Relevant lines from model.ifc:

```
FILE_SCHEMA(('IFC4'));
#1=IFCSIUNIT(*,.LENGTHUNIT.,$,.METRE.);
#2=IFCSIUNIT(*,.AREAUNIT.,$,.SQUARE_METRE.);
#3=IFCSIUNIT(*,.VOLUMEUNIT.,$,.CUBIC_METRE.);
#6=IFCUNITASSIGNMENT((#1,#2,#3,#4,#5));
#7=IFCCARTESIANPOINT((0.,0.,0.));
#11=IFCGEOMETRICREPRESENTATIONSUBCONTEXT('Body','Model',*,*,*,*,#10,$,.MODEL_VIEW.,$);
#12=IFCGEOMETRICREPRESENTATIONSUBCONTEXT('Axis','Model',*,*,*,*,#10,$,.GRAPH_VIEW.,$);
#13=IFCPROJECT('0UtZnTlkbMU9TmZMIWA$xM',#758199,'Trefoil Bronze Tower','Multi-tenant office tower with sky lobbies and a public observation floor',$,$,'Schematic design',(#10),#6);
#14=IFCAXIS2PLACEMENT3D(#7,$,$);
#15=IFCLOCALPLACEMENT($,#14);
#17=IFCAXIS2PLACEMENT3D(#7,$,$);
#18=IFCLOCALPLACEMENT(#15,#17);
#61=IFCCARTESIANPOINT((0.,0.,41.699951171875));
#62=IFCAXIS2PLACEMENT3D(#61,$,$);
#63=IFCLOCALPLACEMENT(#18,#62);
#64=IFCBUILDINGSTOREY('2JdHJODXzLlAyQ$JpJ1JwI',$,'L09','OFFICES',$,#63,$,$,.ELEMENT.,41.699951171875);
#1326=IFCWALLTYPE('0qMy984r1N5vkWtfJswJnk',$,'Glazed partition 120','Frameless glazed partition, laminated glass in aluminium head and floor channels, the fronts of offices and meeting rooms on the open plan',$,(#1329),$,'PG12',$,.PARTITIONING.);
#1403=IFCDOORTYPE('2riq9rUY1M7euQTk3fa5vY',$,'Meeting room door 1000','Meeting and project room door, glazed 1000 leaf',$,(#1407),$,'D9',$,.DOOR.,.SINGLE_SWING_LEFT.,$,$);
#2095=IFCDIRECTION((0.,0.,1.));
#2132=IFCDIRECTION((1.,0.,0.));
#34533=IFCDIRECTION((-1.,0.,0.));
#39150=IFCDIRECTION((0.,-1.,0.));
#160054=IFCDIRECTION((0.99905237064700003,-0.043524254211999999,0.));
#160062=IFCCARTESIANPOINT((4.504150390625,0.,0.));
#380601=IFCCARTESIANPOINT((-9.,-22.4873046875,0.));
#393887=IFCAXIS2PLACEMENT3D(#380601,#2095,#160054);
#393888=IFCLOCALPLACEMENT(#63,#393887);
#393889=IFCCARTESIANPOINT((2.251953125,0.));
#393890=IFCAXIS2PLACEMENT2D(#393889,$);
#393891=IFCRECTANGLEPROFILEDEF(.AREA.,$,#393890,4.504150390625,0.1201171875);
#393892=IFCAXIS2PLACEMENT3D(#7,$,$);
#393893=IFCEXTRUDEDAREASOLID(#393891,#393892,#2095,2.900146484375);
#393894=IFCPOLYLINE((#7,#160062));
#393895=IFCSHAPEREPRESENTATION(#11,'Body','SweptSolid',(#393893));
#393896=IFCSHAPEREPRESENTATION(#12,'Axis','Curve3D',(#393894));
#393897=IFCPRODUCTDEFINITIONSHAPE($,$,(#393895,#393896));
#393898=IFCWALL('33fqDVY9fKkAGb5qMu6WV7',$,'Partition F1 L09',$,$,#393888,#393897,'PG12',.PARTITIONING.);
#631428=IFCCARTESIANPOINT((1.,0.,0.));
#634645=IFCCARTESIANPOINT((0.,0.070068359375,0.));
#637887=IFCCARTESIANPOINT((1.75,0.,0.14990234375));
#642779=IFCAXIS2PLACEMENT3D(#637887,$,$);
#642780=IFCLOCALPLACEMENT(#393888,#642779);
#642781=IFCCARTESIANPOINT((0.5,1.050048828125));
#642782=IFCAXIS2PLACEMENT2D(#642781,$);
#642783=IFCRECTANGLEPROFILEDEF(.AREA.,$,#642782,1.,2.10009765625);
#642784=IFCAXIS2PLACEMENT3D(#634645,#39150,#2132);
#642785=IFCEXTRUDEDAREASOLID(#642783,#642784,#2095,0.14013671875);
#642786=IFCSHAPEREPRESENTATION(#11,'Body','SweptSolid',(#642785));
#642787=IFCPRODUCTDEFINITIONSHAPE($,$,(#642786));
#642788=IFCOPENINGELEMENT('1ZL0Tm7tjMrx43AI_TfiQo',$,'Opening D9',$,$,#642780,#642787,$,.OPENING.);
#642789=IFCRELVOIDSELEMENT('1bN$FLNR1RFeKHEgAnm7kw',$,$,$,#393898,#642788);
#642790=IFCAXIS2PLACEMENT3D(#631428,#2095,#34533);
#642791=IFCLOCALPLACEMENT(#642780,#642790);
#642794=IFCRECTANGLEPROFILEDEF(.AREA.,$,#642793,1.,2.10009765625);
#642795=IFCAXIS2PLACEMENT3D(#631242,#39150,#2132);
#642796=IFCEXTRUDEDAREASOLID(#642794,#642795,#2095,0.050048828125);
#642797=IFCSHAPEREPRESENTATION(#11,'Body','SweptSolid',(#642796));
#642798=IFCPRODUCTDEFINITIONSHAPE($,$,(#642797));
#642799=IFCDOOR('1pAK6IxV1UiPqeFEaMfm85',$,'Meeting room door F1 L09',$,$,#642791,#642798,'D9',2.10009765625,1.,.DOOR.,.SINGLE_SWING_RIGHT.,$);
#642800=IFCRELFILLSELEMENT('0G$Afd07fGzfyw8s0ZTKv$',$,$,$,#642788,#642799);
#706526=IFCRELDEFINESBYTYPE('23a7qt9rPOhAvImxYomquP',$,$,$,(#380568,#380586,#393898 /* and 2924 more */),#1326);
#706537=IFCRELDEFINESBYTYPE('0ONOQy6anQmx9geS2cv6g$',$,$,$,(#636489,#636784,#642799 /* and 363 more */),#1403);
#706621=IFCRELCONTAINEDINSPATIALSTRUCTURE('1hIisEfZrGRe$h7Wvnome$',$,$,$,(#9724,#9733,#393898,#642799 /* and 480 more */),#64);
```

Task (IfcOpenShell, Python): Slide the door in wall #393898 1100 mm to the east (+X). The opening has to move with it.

```python
import ifcopenshell
import ifcopenshell.api.geometry
import ifcopenshell.util.placement
import ifcopenshell.util.unit

model = ifcopenshell.open("model.ifc")
unit_scale = ifcopenshell.util.unit.calculate_unit_scale(model)

door = model.by_guid("1pAK6IxV1UiPqeFEaMfm85")
opening = door.FillsVoids[0].RelatingOpeningElement
wall = opening.VoidsElements[0].RelatingBuildingElement

wall_matrix = ifcopenshell.util.placement.get_local_placement(wall.ObjectPlacement)
shift = wall_matrix[:3, 0] * 1.1 / unit_scale
before = ifcopenshell.util.placement.get_local_placement(door.ObjectPlacement)[:3, 3].copy()

# The door is placed relative to its opening, so it follows when the opening moves.
matrix = ifcopenshell.util.placement.get_local_placement(opening.ObjectPlacement)
matrix[:3, 3] += shift
ifcopenshell.api.geometry.edit_object_placement(
    model, product=opening, matrix=matrix, is_si=False, should_transform_children=True
)

after = ifcopenshell.util.placement.get_local_placement(door.ObjectPlacement)[:3, 3]
print("door moved by", (after - before).round(3) + 0.0)

model.write("model_updated.ifc")
```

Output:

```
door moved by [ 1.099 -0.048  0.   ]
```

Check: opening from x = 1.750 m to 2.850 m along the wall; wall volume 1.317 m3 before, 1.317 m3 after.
